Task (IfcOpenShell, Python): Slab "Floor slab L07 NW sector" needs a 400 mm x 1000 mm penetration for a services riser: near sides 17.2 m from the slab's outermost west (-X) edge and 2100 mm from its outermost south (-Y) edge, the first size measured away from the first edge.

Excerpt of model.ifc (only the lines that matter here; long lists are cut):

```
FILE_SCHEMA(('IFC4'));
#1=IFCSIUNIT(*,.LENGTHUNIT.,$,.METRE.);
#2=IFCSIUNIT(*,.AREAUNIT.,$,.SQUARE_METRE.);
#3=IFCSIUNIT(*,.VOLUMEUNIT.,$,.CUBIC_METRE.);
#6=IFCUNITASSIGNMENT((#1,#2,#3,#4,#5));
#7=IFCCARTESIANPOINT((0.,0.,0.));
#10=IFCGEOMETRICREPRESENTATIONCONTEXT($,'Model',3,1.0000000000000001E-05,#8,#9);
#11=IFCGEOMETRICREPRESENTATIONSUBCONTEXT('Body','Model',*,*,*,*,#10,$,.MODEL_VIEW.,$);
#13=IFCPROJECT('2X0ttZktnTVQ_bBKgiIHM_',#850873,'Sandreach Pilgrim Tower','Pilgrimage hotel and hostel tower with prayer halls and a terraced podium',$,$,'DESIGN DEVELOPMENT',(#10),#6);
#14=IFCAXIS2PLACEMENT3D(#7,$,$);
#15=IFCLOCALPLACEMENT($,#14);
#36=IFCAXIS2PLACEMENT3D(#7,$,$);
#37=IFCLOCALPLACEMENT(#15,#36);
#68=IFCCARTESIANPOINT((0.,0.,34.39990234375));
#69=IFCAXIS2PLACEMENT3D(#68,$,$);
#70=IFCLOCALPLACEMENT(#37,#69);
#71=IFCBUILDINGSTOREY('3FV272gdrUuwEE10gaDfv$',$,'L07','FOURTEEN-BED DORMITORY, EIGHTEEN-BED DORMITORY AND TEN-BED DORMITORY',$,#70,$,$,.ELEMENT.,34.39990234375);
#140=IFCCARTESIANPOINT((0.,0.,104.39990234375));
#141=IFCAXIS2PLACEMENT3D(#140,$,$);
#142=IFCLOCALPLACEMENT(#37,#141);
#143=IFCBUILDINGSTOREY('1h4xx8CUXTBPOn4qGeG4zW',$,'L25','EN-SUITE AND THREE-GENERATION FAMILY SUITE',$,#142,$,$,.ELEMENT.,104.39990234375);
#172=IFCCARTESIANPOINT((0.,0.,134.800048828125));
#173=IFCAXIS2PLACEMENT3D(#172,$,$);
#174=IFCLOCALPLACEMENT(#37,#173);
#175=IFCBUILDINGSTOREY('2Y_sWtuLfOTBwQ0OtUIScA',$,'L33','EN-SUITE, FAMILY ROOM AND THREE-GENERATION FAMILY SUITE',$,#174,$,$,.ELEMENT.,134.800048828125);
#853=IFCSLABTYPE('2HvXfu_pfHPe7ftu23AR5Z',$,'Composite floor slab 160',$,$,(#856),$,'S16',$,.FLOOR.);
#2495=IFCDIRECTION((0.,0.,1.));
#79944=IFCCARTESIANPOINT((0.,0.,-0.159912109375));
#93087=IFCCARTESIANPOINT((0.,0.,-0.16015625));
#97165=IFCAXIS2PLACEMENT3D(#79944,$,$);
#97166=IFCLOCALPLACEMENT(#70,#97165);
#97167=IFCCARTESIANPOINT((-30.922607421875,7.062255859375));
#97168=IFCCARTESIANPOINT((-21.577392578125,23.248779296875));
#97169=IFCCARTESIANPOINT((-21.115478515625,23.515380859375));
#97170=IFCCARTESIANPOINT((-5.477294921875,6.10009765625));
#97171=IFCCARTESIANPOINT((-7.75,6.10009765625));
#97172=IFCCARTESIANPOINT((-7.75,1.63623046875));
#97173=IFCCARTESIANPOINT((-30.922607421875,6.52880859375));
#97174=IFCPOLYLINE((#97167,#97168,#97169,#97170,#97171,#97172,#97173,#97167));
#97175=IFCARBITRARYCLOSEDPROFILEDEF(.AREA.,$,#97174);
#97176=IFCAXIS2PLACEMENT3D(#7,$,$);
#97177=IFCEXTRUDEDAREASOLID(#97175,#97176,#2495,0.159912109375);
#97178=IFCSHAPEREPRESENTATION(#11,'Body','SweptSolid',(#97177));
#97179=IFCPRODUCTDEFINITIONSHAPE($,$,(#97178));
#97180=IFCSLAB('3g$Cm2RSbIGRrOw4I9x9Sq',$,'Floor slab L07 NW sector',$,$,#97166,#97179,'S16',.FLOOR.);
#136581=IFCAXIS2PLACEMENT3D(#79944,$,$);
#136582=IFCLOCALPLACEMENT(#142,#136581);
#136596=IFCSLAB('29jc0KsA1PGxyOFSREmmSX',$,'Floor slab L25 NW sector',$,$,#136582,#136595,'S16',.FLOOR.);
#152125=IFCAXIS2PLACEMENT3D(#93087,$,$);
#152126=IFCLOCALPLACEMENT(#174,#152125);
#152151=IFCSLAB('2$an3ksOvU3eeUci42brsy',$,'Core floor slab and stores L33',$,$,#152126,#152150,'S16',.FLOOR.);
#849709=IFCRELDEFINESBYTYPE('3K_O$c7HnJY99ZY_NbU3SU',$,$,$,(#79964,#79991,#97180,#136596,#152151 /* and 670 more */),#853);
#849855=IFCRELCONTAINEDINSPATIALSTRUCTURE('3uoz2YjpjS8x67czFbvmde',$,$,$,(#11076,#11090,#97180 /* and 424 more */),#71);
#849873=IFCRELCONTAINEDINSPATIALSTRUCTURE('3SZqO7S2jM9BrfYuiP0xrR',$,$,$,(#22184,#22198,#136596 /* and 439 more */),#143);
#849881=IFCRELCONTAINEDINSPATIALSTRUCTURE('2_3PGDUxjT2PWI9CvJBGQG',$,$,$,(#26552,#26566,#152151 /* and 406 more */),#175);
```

```python
import numpy as np
import ifcopenshell
import ifcopenshell.api.feature
import ifcopenshell.api.geometry
import ifcopenshell.api.root
import ifcopenshell.geom
import ifcopenshell.util.placement
import ifcopenshell.util.representation
import ifcopenshell.util.shape
import ifcopenshell.util.unit

model = ifcopenshell.open("model.ifc")
unit_scale = ifcopenshell.util.unit.calculate_unit_scale(model)
settings = ifcopenshell.geom.settings()


def volume(element):
    """Net volume in cubic metres, openings subtracted."""
    shape = ifcopenshell.geom.create_shape(settings, element)
    return ifcopenshell.util.shape.get_volume(shape.geometry)


slab = model.by_guid("3g$Cm2RSbIGRrOw4I9x9Sq")
before = volume(slab)

# Extent in the slab's own axes, in metres. The edges named are its -X and -Y sides.
slab_shape = ifcopenshell.geom.create_shape(settings, slab)
vertices = ifcopenshell.util.shape.get_vertices(slab_shape.geometry)
x_min, y_min, bottom = vertices.min(axis=0)
top = vertices[:, 2].max()

opening = ifcopenshell.api.root.create_entity(model, ifc_class="IfcOpeningElement", name="Services riser opening", predefined_type="OPENING")
context = ifcopenshell.util.representation.get_context(model, "Model", "Body", "MODEL_VIEW")
width, depth = 0.4, 1
outline = [(0.0, 0.0), (width, 0.0), (width, depth), (0.0, depth), (0.0, 0.0)]
# Overshoot both faces by 50 mm so the cut is clean.
shape = ifcopenshell.api.geometry.add_slab_representation(
    model, context=context, depth=top - bottom + 0.1, polyline=outline
)
ifcopenshell.api.geometry.assign_representation(model, product=opening, representation=shape)

matrix = ifcopenshell.util.placement.get_local_placement(slab.ObjectPlacement)
matrix[:, 3] = matrix @ np.append(np.array([x_min + 17.2, y_min + 2.1, bottom - 0.05]) / unit_scale, 1.0)
ifcopenshell.api.geometry.edit_object_placement(model, product=opening, matrix=matrix, is_si=False)
ifcopenshell.api.feature.add_feature(model, feature=opening, element=slab)

after = volume(slab)

print(f"slab volume {before:.3f} -> {after:.3f} m3")

model.write("model_edited.ifc")
```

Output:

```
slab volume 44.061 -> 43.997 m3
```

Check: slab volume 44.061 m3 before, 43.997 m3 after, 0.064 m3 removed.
